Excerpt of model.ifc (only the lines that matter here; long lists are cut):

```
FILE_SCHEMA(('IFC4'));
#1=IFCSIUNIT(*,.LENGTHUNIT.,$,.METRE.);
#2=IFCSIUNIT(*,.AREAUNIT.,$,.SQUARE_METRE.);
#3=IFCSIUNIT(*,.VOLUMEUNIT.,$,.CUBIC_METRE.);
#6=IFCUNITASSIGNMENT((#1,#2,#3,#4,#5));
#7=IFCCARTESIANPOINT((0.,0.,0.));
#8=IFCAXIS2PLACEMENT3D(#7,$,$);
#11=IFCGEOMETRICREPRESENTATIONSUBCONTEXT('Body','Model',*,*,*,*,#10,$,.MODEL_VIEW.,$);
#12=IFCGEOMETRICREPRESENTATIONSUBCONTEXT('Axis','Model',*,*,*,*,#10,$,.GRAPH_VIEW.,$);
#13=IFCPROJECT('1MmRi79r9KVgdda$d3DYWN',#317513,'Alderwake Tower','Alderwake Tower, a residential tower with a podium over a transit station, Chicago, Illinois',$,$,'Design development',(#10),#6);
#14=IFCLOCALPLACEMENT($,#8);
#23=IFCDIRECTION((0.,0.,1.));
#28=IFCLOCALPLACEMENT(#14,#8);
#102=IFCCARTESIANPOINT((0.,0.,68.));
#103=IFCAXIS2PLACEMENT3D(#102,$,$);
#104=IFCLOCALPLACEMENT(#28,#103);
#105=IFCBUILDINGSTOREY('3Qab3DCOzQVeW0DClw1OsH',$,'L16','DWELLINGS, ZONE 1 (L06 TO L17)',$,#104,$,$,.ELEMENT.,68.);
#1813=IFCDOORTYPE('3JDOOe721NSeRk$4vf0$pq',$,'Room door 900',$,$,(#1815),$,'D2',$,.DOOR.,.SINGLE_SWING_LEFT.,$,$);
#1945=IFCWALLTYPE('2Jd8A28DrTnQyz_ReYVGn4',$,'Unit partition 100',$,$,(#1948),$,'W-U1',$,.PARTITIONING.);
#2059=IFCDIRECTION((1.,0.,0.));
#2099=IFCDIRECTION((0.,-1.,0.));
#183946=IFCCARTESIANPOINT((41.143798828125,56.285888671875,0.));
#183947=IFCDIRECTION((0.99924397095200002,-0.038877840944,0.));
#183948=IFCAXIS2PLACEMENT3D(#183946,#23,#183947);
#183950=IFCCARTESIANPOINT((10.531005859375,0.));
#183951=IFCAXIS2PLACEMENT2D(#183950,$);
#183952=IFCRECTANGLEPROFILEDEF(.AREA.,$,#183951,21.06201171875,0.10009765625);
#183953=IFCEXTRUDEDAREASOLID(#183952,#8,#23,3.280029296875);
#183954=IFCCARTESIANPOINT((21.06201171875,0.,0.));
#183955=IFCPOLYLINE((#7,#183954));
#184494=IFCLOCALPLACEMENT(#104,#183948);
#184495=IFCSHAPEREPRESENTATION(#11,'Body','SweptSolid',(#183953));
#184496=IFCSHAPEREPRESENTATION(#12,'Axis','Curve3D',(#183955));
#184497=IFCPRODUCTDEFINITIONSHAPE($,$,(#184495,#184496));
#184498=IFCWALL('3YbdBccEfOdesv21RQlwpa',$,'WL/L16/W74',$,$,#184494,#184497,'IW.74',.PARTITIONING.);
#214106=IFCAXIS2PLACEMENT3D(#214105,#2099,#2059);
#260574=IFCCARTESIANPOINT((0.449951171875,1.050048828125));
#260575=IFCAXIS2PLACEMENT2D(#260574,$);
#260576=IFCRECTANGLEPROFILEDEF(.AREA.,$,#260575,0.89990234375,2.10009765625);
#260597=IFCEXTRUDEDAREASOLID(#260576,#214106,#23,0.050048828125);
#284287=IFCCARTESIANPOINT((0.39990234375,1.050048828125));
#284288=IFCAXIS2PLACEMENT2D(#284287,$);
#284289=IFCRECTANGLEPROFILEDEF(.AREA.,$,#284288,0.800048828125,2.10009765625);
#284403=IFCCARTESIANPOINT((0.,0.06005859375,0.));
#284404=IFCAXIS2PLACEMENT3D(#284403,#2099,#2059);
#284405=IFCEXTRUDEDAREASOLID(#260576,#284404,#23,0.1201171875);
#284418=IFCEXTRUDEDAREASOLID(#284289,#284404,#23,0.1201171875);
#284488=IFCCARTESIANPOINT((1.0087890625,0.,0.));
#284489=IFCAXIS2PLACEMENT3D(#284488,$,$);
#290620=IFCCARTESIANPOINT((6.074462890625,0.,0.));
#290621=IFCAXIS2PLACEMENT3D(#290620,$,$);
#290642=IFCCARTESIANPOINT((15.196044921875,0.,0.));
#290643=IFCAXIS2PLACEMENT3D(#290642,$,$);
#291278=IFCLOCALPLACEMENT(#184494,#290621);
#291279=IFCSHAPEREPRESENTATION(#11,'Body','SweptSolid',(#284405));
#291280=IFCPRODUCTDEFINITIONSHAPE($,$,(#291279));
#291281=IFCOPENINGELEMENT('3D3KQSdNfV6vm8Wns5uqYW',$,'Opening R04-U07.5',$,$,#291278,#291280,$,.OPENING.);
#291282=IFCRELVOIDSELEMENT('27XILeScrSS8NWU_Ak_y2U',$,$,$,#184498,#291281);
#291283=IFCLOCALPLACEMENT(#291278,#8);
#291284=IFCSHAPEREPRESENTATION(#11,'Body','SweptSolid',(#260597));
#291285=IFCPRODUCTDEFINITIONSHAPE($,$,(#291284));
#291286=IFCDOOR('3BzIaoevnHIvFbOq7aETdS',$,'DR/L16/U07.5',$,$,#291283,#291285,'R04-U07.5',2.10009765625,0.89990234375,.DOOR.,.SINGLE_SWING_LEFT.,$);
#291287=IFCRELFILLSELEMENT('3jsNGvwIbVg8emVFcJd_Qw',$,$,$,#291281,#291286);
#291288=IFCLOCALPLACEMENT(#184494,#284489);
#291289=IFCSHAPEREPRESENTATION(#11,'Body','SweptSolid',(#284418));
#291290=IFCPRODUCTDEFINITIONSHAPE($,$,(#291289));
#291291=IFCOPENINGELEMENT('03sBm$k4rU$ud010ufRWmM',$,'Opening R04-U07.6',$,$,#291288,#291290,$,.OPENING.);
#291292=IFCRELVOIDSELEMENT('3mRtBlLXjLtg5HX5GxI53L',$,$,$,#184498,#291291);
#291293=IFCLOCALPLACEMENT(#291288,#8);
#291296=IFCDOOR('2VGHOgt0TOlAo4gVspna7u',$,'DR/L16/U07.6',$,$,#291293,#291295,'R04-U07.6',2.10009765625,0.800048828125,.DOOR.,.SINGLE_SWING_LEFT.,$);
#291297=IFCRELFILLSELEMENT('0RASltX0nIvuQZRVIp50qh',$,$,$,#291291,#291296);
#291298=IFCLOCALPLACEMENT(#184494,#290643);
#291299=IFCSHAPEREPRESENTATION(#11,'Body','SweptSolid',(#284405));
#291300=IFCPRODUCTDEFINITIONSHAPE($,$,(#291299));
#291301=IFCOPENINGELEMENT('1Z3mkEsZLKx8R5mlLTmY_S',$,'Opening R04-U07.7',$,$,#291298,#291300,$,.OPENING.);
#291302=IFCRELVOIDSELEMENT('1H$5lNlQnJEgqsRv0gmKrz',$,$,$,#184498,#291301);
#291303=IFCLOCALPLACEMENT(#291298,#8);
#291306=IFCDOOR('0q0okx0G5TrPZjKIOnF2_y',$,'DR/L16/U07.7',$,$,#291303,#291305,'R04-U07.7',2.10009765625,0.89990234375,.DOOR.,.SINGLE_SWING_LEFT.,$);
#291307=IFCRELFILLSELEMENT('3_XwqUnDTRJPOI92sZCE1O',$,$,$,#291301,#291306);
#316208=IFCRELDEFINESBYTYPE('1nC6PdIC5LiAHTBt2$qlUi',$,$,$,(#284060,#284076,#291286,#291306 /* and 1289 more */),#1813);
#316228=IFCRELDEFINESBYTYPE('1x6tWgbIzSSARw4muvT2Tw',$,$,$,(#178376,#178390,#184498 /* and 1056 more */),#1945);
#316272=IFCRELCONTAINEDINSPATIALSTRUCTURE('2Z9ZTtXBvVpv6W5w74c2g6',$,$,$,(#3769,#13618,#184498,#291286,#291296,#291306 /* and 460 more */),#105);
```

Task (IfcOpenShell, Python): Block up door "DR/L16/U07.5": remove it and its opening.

```python
import ifcopenshell
import ifcopenshell.api.feature
import ifcopenshell.api.root
import ifcopenshell.geom
import ifcopenshell.util.shape

model = ifcopenshell.open("model.ifc")
settings = ifcopenshell.geom.settings()


def volume(element):
    """Net volume in cubic metres, openings subtracted."""
    shape = ifcopenshell.geom.create_shape(settings, element)
    return ifcopenshell.util.shape.get_volume(shape.geometry)


door = model.by_guid("3BzIaoevnHIvFbOq7aETdS")
opening = door.FillsVoids[0].RelatingOpeningElement
wall = opening.VoidsElements[0].RelatingBuildingElement
before = volume(wall)

ifcopenshell.api.root.remove_product(model, product=door)
ifcopenshell.api.feature.remove_feature(model, feature=opening)

after = volume(wall)

print(f"wall volume {before:.3f} -> {after:.3f} m3")

model.write("model_edited.ifc")
```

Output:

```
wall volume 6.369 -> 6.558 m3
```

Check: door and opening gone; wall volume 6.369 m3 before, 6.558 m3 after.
